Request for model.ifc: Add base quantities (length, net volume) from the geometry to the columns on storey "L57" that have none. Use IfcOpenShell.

First a look at what the model holds.

```python
import ifcopenshell
import ifcopenshell.util.element
import ifcopenshell.util.unit

model = ifcopenshell.open("model.ifc")
print(model.schema)
for unit_type in ("LENGTHUNIT", "AREAUNIT", "VOLUMEUNIT"):
    print(unit_type, ifcopenshell.util.unit.calculate_unit_scale(model, unit_type))
storey = next(s for s in model.by_type("IfcBuildingStorey") if s.Name == "L57")
columns = [e for e in ifcopenshell.util.element.get_decomposition(storey) if e.is_a("IfcColumn")]
for e in sorted(columns, key=lambda e: e.id()):
    print(e.id(), e.is_a(), e.Name, list(ifcopenshell.util.element.get_psets(e, qtos_only=True)), sep=" | ")
```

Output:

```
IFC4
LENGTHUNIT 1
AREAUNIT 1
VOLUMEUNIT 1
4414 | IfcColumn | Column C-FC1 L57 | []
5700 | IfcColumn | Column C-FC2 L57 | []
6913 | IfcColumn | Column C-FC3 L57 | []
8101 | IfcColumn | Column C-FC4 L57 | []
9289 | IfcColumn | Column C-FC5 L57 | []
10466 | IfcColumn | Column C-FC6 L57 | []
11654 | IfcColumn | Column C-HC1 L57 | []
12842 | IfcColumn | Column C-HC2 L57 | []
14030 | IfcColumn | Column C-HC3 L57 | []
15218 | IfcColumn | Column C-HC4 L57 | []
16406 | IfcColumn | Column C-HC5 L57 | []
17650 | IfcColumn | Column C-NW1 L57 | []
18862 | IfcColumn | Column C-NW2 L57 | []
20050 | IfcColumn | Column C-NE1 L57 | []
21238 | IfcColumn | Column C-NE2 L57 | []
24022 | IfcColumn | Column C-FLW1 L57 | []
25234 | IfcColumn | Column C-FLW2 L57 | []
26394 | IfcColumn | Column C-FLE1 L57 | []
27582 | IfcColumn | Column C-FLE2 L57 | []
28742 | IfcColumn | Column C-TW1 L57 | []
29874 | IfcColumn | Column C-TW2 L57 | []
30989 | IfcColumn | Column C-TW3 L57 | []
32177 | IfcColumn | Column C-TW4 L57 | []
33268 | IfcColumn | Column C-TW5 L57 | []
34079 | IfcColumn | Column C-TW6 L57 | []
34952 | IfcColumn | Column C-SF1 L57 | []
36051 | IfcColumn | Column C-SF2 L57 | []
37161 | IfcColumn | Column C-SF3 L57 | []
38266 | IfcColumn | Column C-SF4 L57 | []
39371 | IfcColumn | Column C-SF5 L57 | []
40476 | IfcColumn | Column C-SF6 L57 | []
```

```python
import ifcopenshell
import ifcopenshell.api.pset
import ifcopenshell.geom
import ifcopenshell.util.element
import ifcopenshell.util.shape
import ifcopenshell.util.unit

model = ifcopenshell.open("model.ifc")
unit_scale = ifcopenshell.util.unit.calculate_unit_scale(model)
volume_scale = ifcopenshell.util.unit.calculate_unit_scale(model, "VOLUMEUNIT")
settings = ifcopenshell.geom.settings()

storey = next(s for s in model.by_type("IfcBuildingStorey") if s.Name == "L57")
columns = [e for e in ifcopenshell.util.element.get_decomposition(storey) if e.is_a("IfcColumn")]

for e in sorted(columns, key=lambda e: e.id()):
    if ifcopenshell.util.element.get_psets(e, qtos_only=True, should_inherit=False):
        continue
    # Geometry comes back in metres, in the element's own axes.
    shape = ifcopenshell.geom.create_shape(settings, e)
    values = {
        "Length": ifcopenshell.util.shape.get_z(shape.geometry) / unit_scale,
        "NetVolume": ifcopenshell.util.shape.get_volume(shape.geometry) / volume_scale,
    }
    qto = ifcopenshell.api.pset.add_qto(model, product=e, name="Qto_ColumnBaseQuantities")
    ifcopenshell.api.pset.edit_qto(model, qto=qto, properties=values)
    print(e.id(), {k: round(v, 3) for k, v in values.items()})

model.write("model_updated.ifc")
```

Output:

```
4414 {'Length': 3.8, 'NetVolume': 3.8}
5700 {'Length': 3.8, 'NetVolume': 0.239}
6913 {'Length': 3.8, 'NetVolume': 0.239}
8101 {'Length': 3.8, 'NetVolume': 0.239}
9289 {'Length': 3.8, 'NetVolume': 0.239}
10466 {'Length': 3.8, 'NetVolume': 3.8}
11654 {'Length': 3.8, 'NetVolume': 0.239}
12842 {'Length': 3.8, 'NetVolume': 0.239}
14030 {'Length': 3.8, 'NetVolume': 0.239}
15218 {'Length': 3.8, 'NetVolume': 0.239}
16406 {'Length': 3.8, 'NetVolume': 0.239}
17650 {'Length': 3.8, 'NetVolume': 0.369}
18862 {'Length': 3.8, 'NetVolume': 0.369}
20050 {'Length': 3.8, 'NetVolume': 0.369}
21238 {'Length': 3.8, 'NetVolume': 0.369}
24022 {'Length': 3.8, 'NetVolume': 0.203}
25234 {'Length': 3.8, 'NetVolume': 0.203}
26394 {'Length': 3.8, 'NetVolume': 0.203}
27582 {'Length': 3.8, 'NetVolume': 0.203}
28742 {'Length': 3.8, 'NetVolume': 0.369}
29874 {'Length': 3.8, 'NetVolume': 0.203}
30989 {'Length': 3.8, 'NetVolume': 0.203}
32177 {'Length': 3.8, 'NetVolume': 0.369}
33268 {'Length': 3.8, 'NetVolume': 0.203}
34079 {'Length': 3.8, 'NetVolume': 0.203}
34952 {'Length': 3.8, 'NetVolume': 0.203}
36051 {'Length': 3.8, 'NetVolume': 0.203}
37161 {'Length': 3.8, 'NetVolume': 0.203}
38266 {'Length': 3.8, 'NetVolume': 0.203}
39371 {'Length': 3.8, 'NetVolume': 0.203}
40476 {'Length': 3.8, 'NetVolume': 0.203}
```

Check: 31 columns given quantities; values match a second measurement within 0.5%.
